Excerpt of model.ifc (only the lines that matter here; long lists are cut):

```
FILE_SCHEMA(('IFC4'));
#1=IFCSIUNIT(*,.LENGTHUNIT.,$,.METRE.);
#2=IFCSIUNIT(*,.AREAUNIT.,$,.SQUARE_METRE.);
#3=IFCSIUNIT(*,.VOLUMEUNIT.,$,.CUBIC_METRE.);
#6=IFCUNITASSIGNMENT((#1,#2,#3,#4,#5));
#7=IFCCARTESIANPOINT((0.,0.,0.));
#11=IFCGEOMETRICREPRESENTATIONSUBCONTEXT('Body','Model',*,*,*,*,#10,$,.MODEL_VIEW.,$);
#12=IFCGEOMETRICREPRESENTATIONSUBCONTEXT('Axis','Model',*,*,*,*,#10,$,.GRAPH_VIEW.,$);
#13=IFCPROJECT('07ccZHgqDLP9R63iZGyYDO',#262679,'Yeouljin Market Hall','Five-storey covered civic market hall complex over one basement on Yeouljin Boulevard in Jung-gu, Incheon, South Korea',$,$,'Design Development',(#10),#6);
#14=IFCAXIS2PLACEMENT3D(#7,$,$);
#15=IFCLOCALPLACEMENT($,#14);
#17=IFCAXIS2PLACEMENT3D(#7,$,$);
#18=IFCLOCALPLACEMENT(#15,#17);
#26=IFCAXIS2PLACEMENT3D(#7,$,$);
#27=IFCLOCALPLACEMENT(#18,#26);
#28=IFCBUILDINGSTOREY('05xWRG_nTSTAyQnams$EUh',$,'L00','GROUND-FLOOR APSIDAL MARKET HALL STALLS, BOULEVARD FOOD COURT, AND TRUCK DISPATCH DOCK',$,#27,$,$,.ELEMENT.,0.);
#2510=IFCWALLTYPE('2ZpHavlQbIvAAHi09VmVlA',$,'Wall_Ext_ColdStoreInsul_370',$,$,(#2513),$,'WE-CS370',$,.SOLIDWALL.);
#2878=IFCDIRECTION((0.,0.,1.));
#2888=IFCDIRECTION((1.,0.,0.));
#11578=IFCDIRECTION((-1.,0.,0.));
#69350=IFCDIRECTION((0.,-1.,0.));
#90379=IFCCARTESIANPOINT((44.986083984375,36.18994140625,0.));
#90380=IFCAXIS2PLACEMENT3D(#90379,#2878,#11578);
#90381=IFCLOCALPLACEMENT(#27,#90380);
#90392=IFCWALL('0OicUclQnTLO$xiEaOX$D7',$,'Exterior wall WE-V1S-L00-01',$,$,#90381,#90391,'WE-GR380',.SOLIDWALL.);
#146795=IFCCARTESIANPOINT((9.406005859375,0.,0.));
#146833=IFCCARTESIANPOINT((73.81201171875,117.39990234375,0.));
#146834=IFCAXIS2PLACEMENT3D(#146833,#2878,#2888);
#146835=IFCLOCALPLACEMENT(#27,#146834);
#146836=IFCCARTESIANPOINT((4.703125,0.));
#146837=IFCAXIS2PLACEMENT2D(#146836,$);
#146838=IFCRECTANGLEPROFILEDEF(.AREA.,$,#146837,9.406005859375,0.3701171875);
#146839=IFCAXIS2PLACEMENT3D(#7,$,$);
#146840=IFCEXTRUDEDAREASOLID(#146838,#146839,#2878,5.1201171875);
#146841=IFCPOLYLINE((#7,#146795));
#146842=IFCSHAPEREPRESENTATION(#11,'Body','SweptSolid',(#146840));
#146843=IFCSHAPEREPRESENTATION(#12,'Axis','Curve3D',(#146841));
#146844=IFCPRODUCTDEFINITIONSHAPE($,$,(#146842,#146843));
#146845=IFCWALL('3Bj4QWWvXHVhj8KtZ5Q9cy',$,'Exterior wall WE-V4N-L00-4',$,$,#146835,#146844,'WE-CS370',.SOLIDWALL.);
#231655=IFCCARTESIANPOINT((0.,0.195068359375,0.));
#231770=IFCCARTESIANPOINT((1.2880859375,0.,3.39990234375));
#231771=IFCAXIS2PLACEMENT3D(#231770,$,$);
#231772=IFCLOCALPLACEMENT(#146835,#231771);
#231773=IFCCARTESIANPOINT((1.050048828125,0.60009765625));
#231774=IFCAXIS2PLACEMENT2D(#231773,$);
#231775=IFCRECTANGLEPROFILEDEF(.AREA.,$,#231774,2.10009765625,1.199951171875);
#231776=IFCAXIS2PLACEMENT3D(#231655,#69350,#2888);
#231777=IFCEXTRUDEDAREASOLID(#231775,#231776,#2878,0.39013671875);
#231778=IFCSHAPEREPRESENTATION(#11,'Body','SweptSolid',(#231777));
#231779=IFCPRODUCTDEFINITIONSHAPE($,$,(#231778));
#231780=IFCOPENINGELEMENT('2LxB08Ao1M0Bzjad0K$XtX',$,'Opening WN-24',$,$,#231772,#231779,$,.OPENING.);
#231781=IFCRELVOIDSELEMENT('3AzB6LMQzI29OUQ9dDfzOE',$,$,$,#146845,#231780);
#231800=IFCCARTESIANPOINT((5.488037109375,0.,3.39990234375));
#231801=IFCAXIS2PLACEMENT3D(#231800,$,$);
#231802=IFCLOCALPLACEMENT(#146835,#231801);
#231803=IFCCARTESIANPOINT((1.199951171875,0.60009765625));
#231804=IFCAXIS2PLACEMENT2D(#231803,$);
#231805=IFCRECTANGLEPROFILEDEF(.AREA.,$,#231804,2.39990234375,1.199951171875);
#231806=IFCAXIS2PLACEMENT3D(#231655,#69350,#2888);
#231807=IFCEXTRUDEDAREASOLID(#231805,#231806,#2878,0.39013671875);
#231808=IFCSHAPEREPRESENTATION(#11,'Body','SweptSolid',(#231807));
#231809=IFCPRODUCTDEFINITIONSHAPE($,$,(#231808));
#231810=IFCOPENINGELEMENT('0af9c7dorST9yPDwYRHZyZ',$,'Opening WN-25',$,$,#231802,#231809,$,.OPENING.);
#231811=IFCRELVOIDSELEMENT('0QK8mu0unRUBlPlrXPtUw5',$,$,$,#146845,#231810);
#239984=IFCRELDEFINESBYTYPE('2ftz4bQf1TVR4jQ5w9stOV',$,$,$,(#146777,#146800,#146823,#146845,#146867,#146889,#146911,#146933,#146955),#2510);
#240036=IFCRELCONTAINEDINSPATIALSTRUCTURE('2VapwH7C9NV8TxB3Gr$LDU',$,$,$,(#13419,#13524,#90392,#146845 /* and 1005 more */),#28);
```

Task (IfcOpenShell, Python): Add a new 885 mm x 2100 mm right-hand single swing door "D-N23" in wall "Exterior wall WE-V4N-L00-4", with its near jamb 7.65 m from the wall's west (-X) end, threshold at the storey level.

```python
import numpy as np
import ifcopenshell
import ifcopenshell.api.feature
import ifcopenshell.api.geometry
import ifcopenshell.api.root
import ifcopenshell.api.spatial
import ifcopenshell.geom
import ifcopenshell.util.element
import ifcopenshell.util.placement
import ifcopenshell.util.representation
import ifcopenshell.util.shape
import ifcopenshell.util.unit

model = ifcopenshell.open("model.ifc")
unit_scale = ifcopenshell.util.unit.calculate_unit_scale(model)
settings = ifcopenshell.geom.settings()


def volume(element):
    """Net volume in cubic metres, openings subtracted."""
    shape = ifcopenshell.geom.create_shape(settings, element)
    return ifcopenshell.util.shape.get_volume(shape.geometry)


wall = model.by_guid("3Bj4QWWvXHVhj8KtZ5Q9cy")
storey = ifcopenshell.util.element.get_container(wall, ifc_class="IfcBuildingStorey")
context = ifcopenshell.util.representation.get_context(model, "Model", "Body", "MODEL_VIEW")
before = volume(wall)

width, height, from_end, sill = 0.885, 2.1, 7.65, 0.0  # metres

# The wall runs along its own X axis, and the end named is its -X end.
wall_shape = ifcopenshell.geom.create_shape(settings, wall)
x, y, z = ifcopenshell.util.shape.get_vertices(wall_shape.geometry).T
start = x.min() + from_end
face, thickness = float(y.min()), float(y.max() - y.min())
wall_matrix = ifcopenshell.util.placement.get_local_placement(wall.ObjectPlacement)
level = ifcopenshell.util.placement.get_local_placement(storey.ObjectPlacement)[2, 3]


def in_wall(x, y):
    """Placement at x, y metres in the wall's axes, at sill height."""
    matrix = wall_matrix.copy()
    matrix[:, 3] = wall_matrix @ np.array([x / unit_scale, y / unit_scale, 0.0, 1.0])
    matrix[2, 3] = level + sill / unit_scale
    return matrix


# Opening: a box that overshoots both wall faces by 50 mm.
opening = ifcopenshell.api.root.create_entity(model, ifc_class="IfcOpeningElement", predefined_type="OPENING")
box = ifcopenshell.api.geometry.add_wall_representation(
    model, context=context, length=width, height=height, thickness=thickness + 0.1
)
ifcopenshell.api.geometry.assign_representation(model, product=opening, representation=box)
ifcopenshell.api.geometry.edit_object_placement(model, product=opening, matrix=in_wall(start, face - 0.05), is_si=False)
ifcopenshell.api.feature.add_feature(model, feature=opening, element=wall)

door = ifcopenshell.api.root.create_entity(model, ifc_class="IfcDoor", name="D-N23", predefined_type="DOOR")
door.OverallWidth, door.OverallHeight = width / unit_scale, height / unit_scale
door.OperationType = "SINGLE_SWING_RIGHT"
body = ifcopenshell.api.geometry.add_door_representation(
    model,
    context=context,
    overall_width=door.OverallWidth,
    overall_height=door.OverallHeight,
    operation_type="SINGLE_SWING_RIGHT",
    lining_properties={"LiningDepth": thickness / unit_scale, "ThresholdDepth": thickness / unit_scale},
)
ifcopenshell.api.geometry.assign_representation(model, product=door, representation=body)
ifcopenshell.api.spatial.assign_container(model, products=[door], relating_structure=storey)
ifcopenshell.api.feature.add_filling(model, opening=opening, element=door)

# The lining spans the wall, so the door starts at the wall face.
ifcopenshell.api.geometry.edit_object_placement(model, product=door, matrix=in_wall(start, face), is_si=False)

after = volume(wall)

print(f"wall volume {before:.3f} -> {after:.3f} m3")

model.write("model_rev.ifc")
```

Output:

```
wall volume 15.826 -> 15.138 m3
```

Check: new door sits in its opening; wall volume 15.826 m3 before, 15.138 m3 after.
